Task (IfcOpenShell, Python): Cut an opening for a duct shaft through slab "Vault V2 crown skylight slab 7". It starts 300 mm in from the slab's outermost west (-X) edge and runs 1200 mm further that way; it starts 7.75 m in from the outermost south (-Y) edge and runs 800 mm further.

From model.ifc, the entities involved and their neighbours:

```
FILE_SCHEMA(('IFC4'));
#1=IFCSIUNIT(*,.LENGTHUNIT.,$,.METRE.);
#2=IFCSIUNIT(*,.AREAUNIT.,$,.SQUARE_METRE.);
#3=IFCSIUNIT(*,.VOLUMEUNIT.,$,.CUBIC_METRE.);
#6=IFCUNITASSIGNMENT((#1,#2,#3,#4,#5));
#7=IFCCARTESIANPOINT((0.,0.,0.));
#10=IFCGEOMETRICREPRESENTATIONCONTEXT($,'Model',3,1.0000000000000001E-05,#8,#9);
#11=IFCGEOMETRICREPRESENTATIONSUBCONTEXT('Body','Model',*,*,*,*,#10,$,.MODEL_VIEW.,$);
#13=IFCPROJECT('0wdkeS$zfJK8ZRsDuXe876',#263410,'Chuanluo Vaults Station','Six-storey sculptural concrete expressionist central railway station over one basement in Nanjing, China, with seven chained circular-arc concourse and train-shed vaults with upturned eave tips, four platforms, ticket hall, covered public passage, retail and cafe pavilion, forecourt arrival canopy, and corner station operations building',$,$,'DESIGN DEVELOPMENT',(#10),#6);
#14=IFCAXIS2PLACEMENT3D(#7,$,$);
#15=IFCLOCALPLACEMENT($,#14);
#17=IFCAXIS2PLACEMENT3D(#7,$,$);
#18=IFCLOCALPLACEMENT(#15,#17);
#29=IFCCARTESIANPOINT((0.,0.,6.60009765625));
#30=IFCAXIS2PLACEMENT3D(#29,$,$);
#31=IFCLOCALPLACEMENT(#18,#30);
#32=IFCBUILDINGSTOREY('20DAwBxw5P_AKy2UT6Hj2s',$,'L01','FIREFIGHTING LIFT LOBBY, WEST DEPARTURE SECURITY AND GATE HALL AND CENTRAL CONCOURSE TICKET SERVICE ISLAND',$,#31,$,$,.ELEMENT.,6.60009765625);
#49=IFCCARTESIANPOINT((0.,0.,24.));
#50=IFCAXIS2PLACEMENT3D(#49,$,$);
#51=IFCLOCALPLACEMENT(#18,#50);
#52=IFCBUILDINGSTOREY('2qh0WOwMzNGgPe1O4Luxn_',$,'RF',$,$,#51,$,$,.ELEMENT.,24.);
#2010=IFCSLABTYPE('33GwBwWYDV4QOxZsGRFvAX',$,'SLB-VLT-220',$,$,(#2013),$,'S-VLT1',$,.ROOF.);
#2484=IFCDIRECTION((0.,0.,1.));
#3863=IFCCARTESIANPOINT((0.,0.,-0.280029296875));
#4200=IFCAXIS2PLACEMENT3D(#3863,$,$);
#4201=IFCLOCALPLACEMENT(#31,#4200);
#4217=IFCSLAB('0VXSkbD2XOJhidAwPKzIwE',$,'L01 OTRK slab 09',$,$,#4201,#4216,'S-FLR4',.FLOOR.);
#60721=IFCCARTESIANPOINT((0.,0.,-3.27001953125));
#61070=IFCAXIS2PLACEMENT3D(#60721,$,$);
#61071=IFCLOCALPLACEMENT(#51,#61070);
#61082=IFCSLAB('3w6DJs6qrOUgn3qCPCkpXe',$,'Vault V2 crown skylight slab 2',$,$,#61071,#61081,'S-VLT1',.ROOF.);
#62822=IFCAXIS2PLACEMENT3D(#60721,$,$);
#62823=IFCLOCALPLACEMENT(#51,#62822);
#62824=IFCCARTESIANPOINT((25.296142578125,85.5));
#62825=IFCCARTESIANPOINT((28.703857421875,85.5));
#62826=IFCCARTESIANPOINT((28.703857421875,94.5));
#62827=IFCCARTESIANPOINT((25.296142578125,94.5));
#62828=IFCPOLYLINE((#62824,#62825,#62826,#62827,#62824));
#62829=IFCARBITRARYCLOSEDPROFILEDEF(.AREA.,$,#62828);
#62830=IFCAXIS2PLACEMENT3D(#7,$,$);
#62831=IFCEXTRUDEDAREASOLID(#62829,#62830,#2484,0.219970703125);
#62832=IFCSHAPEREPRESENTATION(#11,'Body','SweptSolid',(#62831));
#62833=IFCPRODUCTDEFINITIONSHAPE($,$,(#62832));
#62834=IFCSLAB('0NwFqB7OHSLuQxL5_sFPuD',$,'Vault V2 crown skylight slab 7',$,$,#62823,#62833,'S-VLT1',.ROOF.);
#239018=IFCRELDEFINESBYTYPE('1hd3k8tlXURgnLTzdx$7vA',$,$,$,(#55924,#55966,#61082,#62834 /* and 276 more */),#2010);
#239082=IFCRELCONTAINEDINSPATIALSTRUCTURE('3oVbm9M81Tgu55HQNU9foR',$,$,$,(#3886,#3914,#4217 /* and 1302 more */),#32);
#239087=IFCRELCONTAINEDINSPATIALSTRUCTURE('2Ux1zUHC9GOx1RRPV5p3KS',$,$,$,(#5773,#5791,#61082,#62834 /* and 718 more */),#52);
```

```python
import numpy as np
import ifcopenshell
import ifcopenshell.api.feature
import ifcopenshell.api.geometry
import ifcopenshell.api.root
import ifcopenshell.geom
import ifcopenshell.util.placement
import ifcopenshell.util.representation
import ifcopenshell.util.shape
import ifcopenshell.util.unit

model = ifcopenshell.open("model.ifc")
unit_scale = ifcopenshell.util.unit.calculate_unit_scale(model)
settings = ifcopenshell.geom.settings()


def volume(element):
    """Net volume in cubic metres, openings subtracted."""
    shape = ifcopenshell.geom.create_shape(settings, element)
    return ifcopenshell.util.shape.get_volume(shape.geometry)


slab = model.by_guid("0NwFqB7OHSLuQxL5_sFPuD")
before = volume(slab)

# Extent in the slab's own axes, in metres. The edges named are its -X and -Y sides.
slab_shape = ifcopenshell.geom.create_shape(settings, slab)
vertices = ifcopenshell.util.shape.get_vertices(slab_shape.geometry)
x_min, y_min, bottom = vertices.min(axis=0)
top = vertices[:, 2].max()

opening = ifcopenshell.api.root.create_entity(model, ifc_class="IfcOpeningElement", name="Duct shaft opening", predefined_type="OPENING")
context = ifcopenshell.util.representation.get_context(model, "Model", "Body", "MODEL_VIEW")
width, depth = 1.2, 0.8
outline = [(0.0, 0.0), (width, 0.0), (width, depth), (0.0, depth), (0.0, 0.0)]
# Overshoot both faces by 50 mm so the cut is clean.
shape = ifcopenshell.api.geometry.add_slab_representation(
    model, context=context, depth=top - bottom + 0.1, polyline=outline
)
ifcopenshell.api.geometry.assign_representation(model, product=opening, representation=shape)

matrix = ifcopenshell.util.placement.get_local_placement(slab.ObjectPlacement)
matrix[:, 3] = matrix @ np.append(np.array([x_min + 0.3, y_min + 7.75, bottom - 0.05]) / unit_scale, 1.0)
ifcopenshell.api.geometry.edit_object_placement(model, product=opening, matrix=matrix, is_si=False)
ifcopenshell.api.feature.add_feature(model, feature=opening, element=slab)

after = volume(slab)

print(f"slab volume {before:.3f} -> {after:.3f} m3")

model.write("model_v2.ifc")
```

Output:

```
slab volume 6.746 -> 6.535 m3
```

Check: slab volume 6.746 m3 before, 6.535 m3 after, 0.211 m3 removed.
